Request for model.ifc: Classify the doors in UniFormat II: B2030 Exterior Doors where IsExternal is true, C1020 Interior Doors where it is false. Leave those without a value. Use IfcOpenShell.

First a look at what the model holds.

```python
import ifcopenshell
import ifcopenshell.util.element

model = ifcopenshell.open("model.ifc")
print(model.schema)
print("classifications:", [c.Name for c in model.by_type("IfcClassification")])
values = [ifcopenshell.util.element.get_pset(e, "Pset_DoorCommon", "IsExternal") for e in model.by_type("IfcDoor")]
for value in (True, False, None):
    print("IsExternal", value, values.count(value))
```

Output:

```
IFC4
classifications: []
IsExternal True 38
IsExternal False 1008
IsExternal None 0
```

```python
import ifcopenshell
import ifcopenshell.api.classification
import ifcopenshell.util.element

model = ifcopenshell.open("model.ifc")

system = ifcopenshell.api.classification.add_classification(model, classification="UniFormat II")

doors = model.by_type("IfcDoor")
external = {e: ifcopenshell.util.element.get_pset(e, "Pset_DoorCommon", "IsExternal") for e in doors}
for flag, code, name in ((True, "B2030", "Exterior Doors"), (False, "C1020", "Interior Doors")):
    products = [e for e in doors if external[e] is flag]
    ifcopenshell.api.classification.add_reference(
        model, products=products, classification=system, identification=code, name=name
    )
    print(code, len(products))

model.write("model-out.ifc")
```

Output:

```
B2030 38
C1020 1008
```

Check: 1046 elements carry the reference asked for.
